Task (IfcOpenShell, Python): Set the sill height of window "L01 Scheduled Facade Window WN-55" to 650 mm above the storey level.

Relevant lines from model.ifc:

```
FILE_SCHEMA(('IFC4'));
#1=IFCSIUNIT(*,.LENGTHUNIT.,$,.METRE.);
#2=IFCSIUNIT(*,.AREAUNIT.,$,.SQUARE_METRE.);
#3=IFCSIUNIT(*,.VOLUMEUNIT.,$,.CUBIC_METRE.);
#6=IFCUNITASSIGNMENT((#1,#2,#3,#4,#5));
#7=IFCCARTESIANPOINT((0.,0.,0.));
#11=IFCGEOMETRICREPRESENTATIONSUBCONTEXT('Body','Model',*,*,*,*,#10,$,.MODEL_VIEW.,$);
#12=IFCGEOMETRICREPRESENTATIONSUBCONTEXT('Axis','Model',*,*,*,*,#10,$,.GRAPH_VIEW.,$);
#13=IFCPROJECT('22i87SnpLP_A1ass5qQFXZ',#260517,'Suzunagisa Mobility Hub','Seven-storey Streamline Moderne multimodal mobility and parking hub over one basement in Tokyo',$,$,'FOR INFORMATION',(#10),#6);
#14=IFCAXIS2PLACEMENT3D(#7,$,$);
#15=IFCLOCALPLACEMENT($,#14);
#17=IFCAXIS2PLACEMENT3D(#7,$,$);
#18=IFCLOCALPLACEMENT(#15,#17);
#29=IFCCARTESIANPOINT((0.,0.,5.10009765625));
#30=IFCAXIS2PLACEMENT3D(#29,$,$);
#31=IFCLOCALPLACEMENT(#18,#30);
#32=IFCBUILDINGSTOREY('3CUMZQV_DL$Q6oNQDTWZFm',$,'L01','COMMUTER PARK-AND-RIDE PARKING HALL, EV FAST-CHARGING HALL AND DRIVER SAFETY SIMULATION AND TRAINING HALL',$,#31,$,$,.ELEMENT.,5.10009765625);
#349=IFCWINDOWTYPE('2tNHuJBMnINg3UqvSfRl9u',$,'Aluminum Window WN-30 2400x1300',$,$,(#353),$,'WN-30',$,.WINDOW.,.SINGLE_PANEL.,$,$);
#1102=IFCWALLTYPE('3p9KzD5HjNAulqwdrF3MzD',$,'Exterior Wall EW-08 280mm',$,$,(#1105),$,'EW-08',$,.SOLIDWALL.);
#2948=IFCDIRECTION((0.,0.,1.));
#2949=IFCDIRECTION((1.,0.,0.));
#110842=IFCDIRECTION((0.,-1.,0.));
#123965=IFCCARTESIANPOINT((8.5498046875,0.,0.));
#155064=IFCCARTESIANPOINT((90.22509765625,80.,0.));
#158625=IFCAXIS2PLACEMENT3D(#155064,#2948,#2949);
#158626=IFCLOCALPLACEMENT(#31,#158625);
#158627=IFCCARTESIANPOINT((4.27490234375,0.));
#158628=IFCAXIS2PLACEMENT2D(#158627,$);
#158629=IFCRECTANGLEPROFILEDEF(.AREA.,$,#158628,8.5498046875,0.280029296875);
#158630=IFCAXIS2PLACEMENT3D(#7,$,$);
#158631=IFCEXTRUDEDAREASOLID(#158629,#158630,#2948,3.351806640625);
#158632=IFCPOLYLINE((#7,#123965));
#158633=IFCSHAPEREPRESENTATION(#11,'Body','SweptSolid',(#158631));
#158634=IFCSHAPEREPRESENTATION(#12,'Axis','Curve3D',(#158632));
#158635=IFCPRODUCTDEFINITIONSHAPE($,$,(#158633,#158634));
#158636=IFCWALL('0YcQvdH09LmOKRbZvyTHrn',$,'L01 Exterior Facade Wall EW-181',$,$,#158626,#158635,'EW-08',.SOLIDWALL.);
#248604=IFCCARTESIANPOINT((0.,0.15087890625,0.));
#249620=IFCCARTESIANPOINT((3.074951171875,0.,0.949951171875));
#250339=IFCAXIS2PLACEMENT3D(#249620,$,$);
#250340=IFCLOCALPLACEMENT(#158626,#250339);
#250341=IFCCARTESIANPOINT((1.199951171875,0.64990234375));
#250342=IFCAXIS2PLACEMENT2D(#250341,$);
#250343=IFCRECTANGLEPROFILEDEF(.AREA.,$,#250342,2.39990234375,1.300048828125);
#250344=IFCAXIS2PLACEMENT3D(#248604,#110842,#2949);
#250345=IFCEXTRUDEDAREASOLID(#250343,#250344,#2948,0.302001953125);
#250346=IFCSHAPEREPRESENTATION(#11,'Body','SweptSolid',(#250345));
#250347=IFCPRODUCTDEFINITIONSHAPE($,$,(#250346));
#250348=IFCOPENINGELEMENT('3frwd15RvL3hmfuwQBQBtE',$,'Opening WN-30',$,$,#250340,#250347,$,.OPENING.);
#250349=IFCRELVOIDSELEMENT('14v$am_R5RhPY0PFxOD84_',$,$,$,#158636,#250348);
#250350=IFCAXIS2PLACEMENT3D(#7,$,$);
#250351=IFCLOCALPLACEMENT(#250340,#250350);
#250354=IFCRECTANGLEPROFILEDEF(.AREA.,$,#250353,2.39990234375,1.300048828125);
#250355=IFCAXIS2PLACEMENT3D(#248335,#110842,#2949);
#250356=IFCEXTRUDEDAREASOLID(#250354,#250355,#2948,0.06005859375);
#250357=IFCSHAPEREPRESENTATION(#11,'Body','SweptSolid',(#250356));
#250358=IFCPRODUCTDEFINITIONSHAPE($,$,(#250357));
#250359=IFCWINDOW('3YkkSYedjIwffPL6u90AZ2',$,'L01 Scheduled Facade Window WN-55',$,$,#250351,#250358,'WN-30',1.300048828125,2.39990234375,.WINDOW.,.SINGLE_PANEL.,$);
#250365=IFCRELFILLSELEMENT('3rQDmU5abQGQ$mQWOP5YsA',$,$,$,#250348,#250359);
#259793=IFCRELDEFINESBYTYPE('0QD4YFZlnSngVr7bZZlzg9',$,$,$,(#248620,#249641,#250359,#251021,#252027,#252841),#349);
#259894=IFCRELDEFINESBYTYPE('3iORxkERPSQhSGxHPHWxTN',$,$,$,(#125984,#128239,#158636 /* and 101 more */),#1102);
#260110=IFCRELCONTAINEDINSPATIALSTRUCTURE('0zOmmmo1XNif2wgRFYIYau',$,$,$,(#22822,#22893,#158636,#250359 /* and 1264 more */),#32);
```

```python
import numpy as np
import ifcopenshell
import ifcopenshell.api.geometry
import ifcopenshell.geom
import ifcopenshell.util.element
import ifcopenshell.util.placement
import ifcopenshell.util.shape
import ifcopenshell.util.unit

model = ifcopenshell.open("model.ifc")
unit_scale = ifcopenshell.util.unit.calculate_unit_scale(model)

window = model.by_id(250359)
opening = window.FillsVoids[0].RelatingOpeningElement
storey = ifcopenshell.util.element.get_container(window, ifc_class="IfcBuildingStorey")
level = ifcopenshell.util.placement.get_local_placement(storey.ObjectPlacement)[2, 3]

# The opening's origin need not be at the sill, so measure its lowest point.
shape = ifcopenshell.geom.create_shape(ifcopenshell.geom.settings(), opening)
bottom = ifcopenshell.util.shape.get_shape_bottom_elevation(shape, shape.geometry) / unit_scale
dz = level + 0.65 / unit_scale - bottom

shift = np.array([0.0, 0.0, dz])
# The window is placed relative to its opening, so it follows when the opening moves.
matrix = ifcopenshell.util.placement.get_local_placement(opening.ObjectPlacement)
matrix[:3, 3] += shift
ifcopenshell.api.geometry.edit_object_placement(
    model, product=opening, matrix=matrix, is_si=False, should_transform_children=True
)

print(f"moved by {dz * unit_scale:+.3f} m")

model.write("model_v2.ifc")
```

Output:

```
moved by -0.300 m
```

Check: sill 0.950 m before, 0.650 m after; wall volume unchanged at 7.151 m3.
